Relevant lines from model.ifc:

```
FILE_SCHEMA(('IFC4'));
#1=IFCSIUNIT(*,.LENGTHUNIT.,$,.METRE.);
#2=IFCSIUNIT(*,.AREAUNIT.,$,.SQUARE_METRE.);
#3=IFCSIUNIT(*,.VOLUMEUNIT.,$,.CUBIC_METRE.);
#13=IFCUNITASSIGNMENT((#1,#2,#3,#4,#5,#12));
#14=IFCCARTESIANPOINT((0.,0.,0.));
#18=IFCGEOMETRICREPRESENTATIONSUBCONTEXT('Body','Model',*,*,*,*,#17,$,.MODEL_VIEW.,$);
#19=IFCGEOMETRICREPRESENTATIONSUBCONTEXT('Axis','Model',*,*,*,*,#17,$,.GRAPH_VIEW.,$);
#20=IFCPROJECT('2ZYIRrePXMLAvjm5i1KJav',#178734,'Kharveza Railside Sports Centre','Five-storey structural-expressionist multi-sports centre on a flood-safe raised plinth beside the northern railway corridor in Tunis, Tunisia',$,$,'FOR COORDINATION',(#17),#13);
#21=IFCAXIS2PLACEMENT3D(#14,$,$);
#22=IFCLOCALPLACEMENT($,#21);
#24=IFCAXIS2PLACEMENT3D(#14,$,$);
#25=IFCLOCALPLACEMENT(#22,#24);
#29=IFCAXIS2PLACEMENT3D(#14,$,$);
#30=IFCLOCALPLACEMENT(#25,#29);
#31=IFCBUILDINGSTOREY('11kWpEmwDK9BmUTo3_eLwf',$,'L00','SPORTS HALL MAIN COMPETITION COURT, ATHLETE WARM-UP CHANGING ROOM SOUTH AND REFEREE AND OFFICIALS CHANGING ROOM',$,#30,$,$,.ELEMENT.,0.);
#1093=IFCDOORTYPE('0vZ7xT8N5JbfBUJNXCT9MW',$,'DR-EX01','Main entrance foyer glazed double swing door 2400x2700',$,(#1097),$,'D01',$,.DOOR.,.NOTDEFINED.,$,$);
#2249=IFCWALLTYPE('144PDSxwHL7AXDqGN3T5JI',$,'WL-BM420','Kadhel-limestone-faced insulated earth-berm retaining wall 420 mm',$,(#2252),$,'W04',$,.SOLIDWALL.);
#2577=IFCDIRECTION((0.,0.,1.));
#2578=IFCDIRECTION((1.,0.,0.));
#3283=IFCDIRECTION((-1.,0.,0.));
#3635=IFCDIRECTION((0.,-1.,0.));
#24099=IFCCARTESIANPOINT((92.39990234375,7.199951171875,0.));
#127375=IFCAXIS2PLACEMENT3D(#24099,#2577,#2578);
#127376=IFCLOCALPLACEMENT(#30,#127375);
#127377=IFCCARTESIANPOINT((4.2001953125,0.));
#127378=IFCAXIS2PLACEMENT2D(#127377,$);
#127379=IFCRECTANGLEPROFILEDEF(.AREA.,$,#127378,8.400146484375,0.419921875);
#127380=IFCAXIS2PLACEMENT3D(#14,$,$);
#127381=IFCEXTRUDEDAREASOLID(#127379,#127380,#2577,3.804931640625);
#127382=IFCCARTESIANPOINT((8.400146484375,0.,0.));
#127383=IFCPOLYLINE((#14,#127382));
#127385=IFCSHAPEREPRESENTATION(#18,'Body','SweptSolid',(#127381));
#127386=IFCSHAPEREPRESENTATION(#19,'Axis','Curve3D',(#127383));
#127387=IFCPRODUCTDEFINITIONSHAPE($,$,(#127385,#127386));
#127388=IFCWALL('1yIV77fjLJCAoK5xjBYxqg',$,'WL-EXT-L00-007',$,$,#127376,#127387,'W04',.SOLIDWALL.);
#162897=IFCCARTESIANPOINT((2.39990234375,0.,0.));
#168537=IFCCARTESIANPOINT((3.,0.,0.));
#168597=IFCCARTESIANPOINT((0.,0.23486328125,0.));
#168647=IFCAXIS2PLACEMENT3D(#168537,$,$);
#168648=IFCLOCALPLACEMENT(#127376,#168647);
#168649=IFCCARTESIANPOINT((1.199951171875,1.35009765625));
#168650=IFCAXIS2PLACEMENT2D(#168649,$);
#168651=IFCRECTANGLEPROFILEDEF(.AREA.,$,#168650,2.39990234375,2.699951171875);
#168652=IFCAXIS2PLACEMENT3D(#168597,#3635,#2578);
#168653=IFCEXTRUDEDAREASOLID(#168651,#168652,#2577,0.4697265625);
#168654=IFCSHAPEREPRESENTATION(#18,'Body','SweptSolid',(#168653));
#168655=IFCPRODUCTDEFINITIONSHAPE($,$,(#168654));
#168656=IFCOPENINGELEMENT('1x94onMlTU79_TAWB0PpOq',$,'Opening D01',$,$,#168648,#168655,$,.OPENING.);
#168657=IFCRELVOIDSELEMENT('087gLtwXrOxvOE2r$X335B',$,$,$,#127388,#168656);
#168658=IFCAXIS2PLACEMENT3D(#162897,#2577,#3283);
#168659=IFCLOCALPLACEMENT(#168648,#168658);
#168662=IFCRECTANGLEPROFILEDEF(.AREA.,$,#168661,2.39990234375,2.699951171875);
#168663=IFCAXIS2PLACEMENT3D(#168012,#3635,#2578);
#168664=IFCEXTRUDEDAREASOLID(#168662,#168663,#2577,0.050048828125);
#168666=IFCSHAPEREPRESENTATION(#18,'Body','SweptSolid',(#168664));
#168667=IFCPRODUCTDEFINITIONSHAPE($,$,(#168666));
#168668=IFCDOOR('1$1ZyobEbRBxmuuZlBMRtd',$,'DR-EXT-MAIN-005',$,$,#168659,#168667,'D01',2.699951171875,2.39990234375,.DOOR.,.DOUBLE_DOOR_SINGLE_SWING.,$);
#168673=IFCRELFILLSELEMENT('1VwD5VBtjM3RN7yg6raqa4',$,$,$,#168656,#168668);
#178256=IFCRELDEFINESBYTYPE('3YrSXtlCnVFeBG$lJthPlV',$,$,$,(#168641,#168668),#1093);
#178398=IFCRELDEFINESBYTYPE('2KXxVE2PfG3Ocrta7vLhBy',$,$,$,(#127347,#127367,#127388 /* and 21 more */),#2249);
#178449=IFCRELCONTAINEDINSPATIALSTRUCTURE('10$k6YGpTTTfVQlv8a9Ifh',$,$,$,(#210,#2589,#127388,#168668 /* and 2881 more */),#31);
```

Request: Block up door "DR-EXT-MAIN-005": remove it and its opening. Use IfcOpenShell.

```python
import ifcopenshell
import ifcopenshell.api.feature
import ifcopenshell.api.root
import ifcopenshell.geom
import ifcopenshell.util.shape

model = ifcopenshell.open("model.ifc")
settings = ifcopenshell.geom.settings()


def volume(element):
    """Net volume in cubic metres, openings subtracted."""
    shape = ifcopenshell.geom.create_shape(settings, element)
    return ifcopenshell.util.shape.get_volume(shape.geometry)


door = model.by_guid("1$1ZyobEbRBxmuuZlBMRtd")
opening = door.FillsVoids[0].RelatingOpeningElement
wall = opening.VoidsElements[0].RelatingBuildingElement
before = volume(wall)

ifcopenshell.api.root.remove_product(model, product=door)
ifcopenshell.api.feature.remove_feature(model, feature=opening)

after = volume(wall)

print(f"wall volume {before:.3f} -> {after:.3f} m3")

model.write("model_updated.ifc")
```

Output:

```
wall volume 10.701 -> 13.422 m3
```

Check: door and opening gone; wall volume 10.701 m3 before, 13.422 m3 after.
